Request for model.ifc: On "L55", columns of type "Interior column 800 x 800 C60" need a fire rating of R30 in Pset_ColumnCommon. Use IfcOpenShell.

First a look at what the model holds.

```python
import ifcopenshell
import ifcopenshell.util.element

model = ifcopenshell.open("model.ifc")
print(model.schema)
storey = next(s for s in model.by_type("IfcBuildingStorey") if s.Name == "L55")
columns = [e for e in ifcopenshell.util.element.get_decomposition(storey) if e.is_a("IfcColumn")]
seen = {}
for e in columns:
    element_type = ifcopenshell.util.element.get_type(e)
    key = (element_type.Name if element_type != e and element_type else None, ifcopenshell.util.element.get_pset(e, "Pset_ColumnCommon", "FireRating"))
    seen[key] = seen.get(key, 0) + 1
for (name, value), count in sorted(seen.items(), key=str):
    print(count, "x", name, "|", value)
```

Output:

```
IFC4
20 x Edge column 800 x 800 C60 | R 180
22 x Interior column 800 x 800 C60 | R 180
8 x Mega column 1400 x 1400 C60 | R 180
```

```python
import ifcopenshell
import ifcopenshell.api.pset
import ifcopenshell.util.element

model = ifcopenshell.open("model.ifc")

storey = next(s for s in model.by_type("IfcBuildingStorey") if s.Name == "L55")
columns = [e for e in ifcopenshell.util.element.get_decomposition(storey) if e.is_a("IfcColumn")]

count = 0
for e in columns:
    element_type = ifcopenshell.util.element.get_type(e)
    if element_type in (None, e) or element_type.Name != "Interior column 800 x 800 C60":
        continue
    found = ifcopenshell.util.element.get_pset(e, "Pset_ColumnCommon", should_inherit=False)
    if found:
        pset = model.by_id(found["id"])
        if len(ifcopenshell.util.element.get_elements_by_pset(pset)) > 1:
            pset = ifcopenshell.api.pset.unshare_pset(model, products=[e], pset=pset)[0]
    else:
        pset = ifcopenshell.api.pset.add_pset(model, product=e, name="Pset_ColumnCommon")
    ifcopenshell.api.pset.edit_pset(model, pset=pset, properties={"FireRating": "R30"})
    count += 1

print(count, "columns updated")

model.write("model_rev.ifc")
```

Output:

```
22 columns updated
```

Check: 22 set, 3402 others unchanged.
